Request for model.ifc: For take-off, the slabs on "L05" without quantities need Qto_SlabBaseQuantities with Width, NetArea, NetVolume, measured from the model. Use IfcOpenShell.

First a look at what the model holds.

```python
import ifcopenshell
import ifcopenshell.util.element
import ifcopenshell.util.unit

model = ifcopenshell.open("model.ifc")
print(model.schema)
for unit_type in ("LENGTHUNIT", "AREAUNIT", "VOLUMEUNIT"):
    print(unit_type, ifcopenshell.util.unit.calculate_unit_scale(model, unit_type))
storey = next(s for s in model.by_type("IfcBuildingStorey") if s.Name == "L05")
slabs = [e for e in ifcopenshell.util.element.get_decomposition(storey) if e.is_a("IfcSlab")]
for e in sorted(slabs, key=lambda e: e.id()):
    print(e.id(), e.is_a(), e.Name, list(ifcopenshell.util.element.get_psets(e, qtos_only=True)), sep=" | ")
```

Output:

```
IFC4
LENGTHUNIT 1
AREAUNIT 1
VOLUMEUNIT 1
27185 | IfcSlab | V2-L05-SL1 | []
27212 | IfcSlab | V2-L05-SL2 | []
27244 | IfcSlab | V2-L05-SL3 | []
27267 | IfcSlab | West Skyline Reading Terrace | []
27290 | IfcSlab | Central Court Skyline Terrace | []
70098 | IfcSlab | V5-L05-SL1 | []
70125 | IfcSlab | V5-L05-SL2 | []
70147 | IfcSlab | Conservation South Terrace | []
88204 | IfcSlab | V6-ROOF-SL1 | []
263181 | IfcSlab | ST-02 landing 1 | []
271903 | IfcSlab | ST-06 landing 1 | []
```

```python
import ifcopenshell
import ifcopenshell.api.pset
import ifcopenshell.geom
import ifcopenshell.util.element
import ifcopenshell.util.shape
import ifcopenshell.util.unit

model = ifcopenshell.open("model.ifc")
unit_scale = ifcopenshell.util.unit.calculate_unit_scale(model)
area_scale = ifcopenshell.util.unit.calculate_unit_scale(model, "AREAUNIT")
volume_scale = ifcopenshell.util.unit.calculate_unit_scale(model, "VOLUMEUNIT")
settings = ifcopenshell.geom.settings()

storey = next(s for s in model.by_type("IfcBuildingStorey") if s.Name == "L05")
slabs = [e for e in ifcopenshell.util.element.get_decomposition(storey) if e.is_a("IfcSlab")]

for e in sorted(slabs, key=lambda e: e.id()):
    if ifcopenshell.util.element.get_psets(e, qtos_only=True, should_inherit=False):
        continue
    # Geometry comes back in metres, in the element's own axes.
    shape = ifcopenshell.geom.create_shape(settings, e)
    values = {
        "Width": ifcopenshell.util.shape.get_z(shape.geometry) / unit_scale,
        "NetArea": ifcopenshell.util.shape.get_footprint_area(shape.geometry) / area_scale,
        "NetVolume": ifcopenshell.util.shape.get_volume(shape.geometry) / volume_scale,
    }
    qto = ifcopenshell.api.pset.add_qto(model, product=e, name="Qto_SlabBaseQuantities")
    ifcopenshell.api.pset.edit_qto(model, qto=qto, properties=values)
    print(e.id(), {k: round(v, 3) for k, v in values.items()})

model.write("model_v2.ifc")
```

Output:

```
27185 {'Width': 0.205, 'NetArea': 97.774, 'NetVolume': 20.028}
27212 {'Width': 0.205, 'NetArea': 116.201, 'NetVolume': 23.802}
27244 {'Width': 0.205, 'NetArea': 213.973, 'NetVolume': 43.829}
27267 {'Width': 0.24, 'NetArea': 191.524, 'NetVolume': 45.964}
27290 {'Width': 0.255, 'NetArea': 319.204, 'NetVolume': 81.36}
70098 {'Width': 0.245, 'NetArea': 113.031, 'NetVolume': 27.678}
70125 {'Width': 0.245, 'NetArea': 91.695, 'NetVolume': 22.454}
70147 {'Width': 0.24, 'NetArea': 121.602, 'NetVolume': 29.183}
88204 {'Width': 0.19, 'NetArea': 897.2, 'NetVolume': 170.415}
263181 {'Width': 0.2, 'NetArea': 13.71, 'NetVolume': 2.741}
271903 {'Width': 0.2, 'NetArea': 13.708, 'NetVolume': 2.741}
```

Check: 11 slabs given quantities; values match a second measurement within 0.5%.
